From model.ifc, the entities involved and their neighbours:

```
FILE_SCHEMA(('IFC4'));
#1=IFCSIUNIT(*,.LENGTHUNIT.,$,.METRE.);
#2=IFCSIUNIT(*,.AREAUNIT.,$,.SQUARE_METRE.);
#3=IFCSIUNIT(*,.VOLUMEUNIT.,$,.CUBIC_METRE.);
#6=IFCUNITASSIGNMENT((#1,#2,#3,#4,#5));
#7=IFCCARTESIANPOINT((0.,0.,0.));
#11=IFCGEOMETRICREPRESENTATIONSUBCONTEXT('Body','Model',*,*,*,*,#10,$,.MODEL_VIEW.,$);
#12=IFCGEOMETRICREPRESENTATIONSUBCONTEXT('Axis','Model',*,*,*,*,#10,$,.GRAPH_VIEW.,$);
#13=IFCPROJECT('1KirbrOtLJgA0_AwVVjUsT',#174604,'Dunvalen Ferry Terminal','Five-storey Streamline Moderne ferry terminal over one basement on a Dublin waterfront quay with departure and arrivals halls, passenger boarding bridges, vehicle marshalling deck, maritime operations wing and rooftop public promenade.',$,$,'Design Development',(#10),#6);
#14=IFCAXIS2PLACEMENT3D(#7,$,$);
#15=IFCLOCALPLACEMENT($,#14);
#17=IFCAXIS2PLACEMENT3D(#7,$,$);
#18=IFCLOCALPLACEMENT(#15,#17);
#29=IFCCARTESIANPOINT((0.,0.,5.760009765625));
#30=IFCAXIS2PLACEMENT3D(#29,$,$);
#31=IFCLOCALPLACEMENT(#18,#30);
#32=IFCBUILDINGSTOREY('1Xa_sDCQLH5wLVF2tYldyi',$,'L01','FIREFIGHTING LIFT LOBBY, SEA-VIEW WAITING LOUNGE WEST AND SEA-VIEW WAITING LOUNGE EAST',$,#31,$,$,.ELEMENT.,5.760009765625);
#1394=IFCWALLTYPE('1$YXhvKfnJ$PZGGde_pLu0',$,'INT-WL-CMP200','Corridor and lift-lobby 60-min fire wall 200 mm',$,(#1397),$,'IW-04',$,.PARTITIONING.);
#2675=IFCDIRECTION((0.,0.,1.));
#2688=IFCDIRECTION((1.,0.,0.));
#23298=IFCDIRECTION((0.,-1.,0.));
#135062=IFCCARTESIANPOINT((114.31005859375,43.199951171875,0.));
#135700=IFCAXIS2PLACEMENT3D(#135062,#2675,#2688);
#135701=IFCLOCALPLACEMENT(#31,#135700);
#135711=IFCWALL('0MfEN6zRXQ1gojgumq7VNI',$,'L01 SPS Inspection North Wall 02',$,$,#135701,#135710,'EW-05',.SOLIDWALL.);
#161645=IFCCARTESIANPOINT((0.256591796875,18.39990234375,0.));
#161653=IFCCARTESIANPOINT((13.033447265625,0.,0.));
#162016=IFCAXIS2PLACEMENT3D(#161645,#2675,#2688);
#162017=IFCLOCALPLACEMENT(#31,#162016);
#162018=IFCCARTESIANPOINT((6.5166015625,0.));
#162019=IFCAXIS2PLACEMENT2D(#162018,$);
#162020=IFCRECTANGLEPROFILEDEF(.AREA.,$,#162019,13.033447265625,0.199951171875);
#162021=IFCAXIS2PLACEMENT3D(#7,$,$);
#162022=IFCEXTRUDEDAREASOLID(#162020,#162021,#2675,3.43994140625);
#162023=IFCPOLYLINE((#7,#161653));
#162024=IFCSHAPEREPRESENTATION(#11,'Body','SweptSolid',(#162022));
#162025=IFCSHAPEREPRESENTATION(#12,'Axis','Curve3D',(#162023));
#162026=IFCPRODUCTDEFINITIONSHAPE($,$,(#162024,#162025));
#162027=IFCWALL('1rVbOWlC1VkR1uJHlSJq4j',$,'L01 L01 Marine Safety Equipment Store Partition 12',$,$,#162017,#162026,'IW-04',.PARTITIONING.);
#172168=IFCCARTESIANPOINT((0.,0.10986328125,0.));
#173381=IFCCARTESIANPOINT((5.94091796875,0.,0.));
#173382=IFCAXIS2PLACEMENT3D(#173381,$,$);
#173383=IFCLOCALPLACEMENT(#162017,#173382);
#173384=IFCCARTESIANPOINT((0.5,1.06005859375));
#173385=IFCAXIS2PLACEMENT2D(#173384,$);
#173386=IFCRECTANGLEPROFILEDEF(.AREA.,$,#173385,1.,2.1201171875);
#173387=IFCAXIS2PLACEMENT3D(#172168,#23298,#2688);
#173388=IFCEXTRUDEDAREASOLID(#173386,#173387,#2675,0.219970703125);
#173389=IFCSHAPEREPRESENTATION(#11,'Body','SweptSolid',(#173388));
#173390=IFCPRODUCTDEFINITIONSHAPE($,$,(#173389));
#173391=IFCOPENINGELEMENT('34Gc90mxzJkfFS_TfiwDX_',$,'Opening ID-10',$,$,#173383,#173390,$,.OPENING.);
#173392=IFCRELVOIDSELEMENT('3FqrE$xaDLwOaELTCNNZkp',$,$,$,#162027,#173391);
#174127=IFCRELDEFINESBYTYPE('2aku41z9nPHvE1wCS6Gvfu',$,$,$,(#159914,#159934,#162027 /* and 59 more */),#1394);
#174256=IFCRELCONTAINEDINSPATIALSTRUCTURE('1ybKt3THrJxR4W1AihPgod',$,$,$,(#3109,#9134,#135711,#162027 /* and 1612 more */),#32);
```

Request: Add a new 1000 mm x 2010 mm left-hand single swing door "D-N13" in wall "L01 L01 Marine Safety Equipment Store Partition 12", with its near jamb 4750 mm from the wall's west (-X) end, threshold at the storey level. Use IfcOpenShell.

```python
import numpy as np
import ifcopenshell
import ifcopenshell.api.feature
import ifcopenshell.api.geometry
import ifcopenshell.api.root
import ifcopenshell.api.spatial
import ifcopenshell.geom
import ifcopenshell.util.element
import ifcopenshell.util.placement
import ifcopenshell.util.representation
import ifcopenshell.util.shape
import ifcopenshell.util.unit

model = ifcopenshell.open("model.ifc")
unit_scale = ifcopenshell.util.unit.calculate_unit_scale(model)
settings = ifcopenshell.geom.settings()


def volume(element):
    """Net volume in cubic metres, openings subtracted."""
    shape = ifcopenshell.geom.create_shape(settings, element)
    return ifcopenshell.util.shape.get_volume(shape.geometry)


wall = model.by_guid("1rVbOWlC1VkR1uJHlSJq4j")
storey = ifcopenshell.util.element.get_container(wall, ifc_class="IfcBuildingStorey")
context = ifcopenshell.util.representation.get_context(model, "Model", "Body", "MODEL_VIEW")
before = volume(wall)

width, height, from_end, sill = 1, 2.01, 4.75, 0.0  # metres

# The wall runs along its own X axis, and the end named is its -X end.
wall_shape = ifcopenshell.geom.create_shape(settings, wall)
x, y, z = ifcopenshell.util.shape.get_vertices(wall_shape.geometry).T
start = x.min() + from_end
face, thickness = float(y.min()), float(y.max() - y.min())
wall_matrix = ifcopenshell.util.placement.get_local_placement(wall.ObjectPlacement)
level = ifcopenshell.util.placement.get_local_placement(storey.ObjectPlacement)[2, 3]


def in_wall(x, y):
    """Placement at x, y metres in the wall's axes, at sill height."""
    matrix = wall_matrix.copy()
    matrix[:, 3] = wall_matrix @ np.array([x / unit_scale, y / unit_scale, 0.0, 1.0])
    matrix[2, 3] = level + sill / unit_scale
    return matrix


# Opening: a box that overshoots both wall faces by 50 mm.
opening = ifcopenshell.api.root.create_entity(model, ifc_class="IfcOpeningElement", predefined_type="OPENING")
box = ifcopenshell.api.geometry.add_wall_representation(
    model, context=context, length=width, height=height, thickness=thickness + 0.1
)
ifcopenshell.api.geometry.assign_representation(model, product=opening, representation=box)
ifcopenshell.api.geometry.edit_object_placement(model, product=opening, matrix=in_wall(start, face - 0.05), is_si=False)
ifcopenshell.api.feature.add_feature(model, feature=opening, element=wall)

door = ifcopenshell.api.root.create_entity(model, ifc_class="IfcDoor", name="D-N13", predefined_type="DOOR")
door.OverallWidth, door.OverallHeight = width / unit_scale, height / unit_scale
door.OperationType = "SINGLE_SWING_LEFT"
body = ifcopenshell.api.geometry.add_door_representation(
    model,
    context=context,
    overall_width=door.OverallWidth,
    overall_height=door.OverallHeight,
    operation_type="SINGLE_SWING_LEFT",
    lining_properties={"LiningDepth": thickness / unit_scale, "ThresholdDepth": thickness / unit_scale},
)
ifcopenshell.api.geometry.assign_representation(model, product=door, representation=body)
ifcopenshell.api.spatial.assign_container(model, products=[door], relating_structure=storey)
ifcopenshell.api.feature.add_filling(model, opening=opening, element=door)

# The lining spans the wall, so the door starts at the wall face.
ifcopenshell.api.geometry.edit_object_placement(model, product=door, matrix=in_wall(start, face), is_si=False)

after = volume(wall)

print(f"wall volume {before:.3f} -> {after:.3f} m3")

model.write("model-out.ifc")
```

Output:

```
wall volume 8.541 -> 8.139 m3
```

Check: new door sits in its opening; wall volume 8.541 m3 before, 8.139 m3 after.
